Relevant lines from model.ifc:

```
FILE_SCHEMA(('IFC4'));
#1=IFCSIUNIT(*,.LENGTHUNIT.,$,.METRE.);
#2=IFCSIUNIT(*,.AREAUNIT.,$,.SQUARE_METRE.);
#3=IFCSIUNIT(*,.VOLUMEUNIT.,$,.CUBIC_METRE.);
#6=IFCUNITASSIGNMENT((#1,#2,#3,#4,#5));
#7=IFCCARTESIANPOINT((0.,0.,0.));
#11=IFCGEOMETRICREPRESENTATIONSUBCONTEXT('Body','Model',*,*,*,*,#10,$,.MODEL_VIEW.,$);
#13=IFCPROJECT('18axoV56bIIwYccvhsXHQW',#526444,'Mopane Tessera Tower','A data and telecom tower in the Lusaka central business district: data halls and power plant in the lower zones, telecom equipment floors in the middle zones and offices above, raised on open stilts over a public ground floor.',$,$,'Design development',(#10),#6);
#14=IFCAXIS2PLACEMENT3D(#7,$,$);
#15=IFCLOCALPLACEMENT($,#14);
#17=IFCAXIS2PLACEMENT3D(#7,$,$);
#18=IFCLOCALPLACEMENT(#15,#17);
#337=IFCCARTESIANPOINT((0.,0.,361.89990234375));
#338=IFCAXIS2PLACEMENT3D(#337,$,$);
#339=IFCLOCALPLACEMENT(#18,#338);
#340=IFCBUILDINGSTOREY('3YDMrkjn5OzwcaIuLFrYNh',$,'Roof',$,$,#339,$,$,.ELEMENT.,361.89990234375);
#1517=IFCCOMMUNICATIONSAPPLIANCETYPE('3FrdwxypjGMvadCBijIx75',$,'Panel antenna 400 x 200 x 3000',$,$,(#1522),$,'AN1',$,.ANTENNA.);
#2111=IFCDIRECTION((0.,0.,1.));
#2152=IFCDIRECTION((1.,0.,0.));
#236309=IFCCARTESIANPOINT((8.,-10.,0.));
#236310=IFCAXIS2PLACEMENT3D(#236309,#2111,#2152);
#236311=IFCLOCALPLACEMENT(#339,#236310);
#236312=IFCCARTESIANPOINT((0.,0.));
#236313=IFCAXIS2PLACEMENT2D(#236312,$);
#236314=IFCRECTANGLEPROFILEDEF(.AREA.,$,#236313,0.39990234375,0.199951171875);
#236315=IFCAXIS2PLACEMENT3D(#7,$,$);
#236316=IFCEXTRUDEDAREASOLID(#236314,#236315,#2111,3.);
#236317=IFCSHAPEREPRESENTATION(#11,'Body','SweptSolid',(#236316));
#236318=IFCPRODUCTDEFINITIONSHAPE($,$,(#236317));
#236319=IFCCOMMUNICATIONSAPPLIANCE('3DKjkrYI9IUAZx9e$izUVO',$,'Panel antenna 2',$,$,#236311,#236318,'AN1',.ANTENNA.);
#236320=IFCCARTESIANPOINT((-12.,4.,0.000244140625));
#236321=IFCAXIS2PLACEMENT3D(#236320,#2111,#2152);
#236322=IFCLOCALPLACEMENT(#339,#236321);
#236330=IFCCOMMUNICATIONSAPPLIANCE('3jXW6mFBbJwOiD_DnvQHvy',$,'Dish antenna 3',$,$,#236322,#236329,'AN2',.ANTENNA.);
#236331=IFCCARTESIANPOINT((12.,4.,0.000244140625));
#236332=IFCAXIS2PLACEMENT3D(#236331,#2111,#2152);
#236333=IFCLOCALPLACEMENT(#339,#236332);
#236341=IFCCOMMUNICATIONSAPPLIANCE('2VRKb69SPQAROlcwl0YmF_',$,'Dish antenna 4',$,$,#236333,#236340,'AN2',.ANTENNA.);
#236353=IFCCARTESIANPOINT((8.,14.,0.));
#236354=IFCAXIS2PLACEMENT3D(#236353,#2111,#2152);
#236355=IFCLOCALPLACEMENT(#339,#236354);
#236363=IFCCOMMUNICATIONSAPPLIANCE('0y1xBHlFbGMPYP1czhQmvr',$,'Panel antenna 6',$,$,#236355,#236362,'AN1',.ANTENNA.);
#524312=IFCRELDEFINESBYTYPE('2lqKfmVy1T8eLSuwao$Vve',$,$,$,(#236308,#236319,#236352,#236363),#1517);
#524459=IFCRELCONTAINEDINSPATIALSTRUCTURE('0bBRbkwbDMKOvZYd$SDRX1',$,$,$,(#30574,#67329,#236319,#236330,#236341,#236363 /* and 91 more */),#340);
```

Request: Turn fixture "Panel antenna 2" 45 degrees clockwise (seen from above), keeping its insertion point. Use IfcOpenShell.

```python
import ifcopenshell
import ifcopenshell.api.geometry
import ifcopenshell.util.placement

model = ifcopenshell.open("model.ifc")

item = model.by_guid("3DKjkrYI9IUAZx9e$izUVO")
matrix = ifcopenshell.util.placement.get_local_placement(item.ObjectPlacement)
matrix = matrix @ ifcopenshell.util.placement.rotation(-45, "Z")
ifcopenshell.api.geometry.edit_object_placement(model, product=item, matrix=matrix, is_si=False)

print(ifcopenshell.util.placement.get_local_placement(item.ObjectPlacement).round(3) + 0.0)

model.write("model_updated.ifc")
```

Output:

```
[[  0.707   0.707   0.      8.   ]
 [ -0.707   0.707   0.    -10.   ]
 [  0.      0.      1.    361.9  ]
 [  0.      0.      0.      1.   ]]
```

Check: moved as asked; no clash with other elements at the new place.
